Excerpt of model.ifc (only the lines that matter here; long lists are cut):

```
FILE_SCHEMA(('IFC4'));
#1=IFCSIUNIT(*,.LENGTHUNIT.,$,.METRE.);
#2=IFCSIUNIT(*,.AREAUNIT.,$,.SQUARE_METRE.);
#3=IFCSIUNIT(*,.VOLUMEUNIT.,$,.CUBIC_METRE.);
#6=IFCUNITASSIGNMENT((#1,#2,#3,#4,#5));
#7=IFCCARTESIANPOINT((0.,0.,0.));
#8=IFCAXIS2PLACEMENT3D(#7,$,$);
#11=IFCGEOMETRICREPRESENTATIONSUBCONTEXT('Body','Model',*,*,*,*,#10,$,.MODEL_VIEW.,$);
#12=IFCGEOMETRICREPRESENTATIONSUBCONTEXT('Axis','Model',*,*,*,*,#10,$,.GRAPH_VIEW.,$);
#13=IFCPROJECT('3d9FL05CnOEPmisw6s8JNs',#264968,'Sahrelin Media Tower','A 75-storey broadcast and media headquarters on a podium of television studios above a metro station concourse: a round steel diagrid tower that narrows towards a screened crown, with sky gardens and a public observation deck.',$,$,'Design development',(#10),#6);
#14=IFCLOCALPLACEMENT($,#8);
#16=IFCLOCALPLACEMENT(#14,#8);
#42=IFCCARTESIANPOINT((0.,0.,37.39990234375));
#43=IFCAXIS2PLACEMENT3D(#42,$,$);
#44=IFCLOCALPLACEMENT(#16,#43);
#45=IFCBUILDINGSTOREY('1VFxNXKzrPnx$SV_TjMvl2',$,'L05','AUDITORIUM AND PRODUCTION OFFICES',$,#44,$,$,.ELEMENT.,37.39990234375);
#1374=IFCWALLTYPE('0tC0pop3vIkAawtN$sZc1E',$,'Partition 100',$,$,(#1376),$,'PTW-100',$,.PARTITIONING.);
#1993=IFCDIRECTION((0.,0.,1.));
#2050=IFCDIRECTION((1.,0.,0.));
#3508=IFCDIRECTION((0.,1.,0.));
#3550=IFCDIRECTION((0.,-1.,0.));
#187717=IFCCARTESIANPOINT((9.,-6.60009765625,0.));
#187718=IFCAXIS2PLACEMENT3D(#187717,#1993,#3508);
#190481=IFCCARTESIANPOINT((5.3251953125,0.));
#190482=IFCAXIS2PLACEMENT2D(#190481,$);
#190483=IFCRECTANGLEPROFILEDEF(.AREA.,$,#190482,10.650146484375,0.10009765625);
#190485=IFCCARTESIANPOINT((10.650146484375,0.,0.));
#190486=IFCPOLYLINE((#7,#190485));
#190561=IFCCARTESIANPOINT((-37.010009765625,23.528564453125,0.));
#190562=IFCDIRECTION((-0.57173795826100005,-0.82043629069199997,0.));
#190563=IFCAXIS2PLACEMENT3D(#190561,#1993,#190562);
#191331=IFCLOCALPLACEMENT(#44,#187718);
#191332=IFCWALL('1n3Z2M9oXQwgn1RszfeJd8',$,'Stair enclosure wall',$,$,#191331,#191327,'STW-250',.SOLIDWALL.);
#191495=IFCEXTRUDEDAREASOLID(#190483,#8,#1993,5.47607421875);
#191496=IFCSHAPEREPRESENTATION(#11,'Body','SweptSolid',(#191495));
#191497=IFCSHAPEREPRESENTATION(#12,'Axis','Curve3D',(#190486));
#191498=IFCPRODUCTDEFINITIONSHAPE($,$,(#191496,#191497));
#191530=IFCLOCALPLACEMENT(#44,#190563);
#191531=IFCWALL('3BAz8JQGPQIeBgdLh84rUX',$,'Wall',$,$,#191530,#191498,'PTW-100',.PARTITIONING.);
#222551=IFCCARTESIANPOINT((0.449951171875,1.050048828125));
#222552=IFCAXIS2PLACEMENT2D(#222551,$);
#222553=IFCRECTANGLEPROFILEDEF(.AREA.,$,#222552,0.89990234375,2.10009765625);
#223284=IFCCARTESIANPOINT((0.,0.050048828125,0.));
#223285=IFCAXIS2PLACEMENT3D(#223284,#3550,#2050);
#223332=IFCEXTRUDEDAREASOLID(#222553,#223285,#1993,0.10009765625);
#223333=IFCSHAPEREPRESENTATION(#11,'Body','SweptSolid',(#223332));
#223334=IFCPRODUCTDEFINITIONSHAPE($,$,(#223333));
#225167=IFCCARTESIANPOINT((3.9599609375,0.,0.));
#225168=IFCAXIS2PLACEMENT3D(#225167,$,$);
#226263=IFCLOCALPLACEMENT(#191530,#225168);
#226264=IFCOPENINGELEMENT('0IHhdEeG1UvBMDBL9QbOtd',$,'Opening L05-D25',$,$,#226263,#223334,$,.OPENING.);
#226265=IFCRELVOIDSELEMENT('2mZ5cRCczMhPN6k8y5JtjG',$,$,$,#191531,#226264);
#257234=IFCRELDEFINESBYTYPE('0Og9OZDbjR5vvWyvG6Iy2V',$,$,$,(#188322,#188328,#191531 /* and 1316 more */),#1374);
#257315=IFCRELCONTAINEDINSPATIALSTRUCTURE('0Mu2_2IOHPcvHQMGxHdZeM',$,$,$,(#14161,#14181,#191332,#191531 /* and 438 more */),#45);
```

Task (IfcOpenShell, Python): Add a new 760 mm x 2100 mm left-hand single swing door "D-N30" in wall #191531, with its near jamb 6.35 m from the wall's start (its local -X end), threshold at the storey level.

```python
import numpy as np
import ifcopenshell
import ifcopenshell.api.feature
import ifcopenshell.api.geometry
import ifcopenshell.api.root
import ifcopenshell.api.spatial
import ifcopenshell.geom
import ifcopenshell.util.element
import ifcopenshell.util.placement
import ifcopenshell.util.representation
import ifcopenshell.util.shape
import ifcopenshell.util.unit

model = ifcopenshell.open("model.ifc")
unit_scale = ifcopenshell.util.unit.calculate_unit_scale(model)
settings = ifcopenshell.geom.settings()


def volume(element):
    """Net volume in cubic metres, openings subtracted."""
    shape = ifcopenshell.geom.create_shape(settings, element)
    return ifcopenshell.util.shape.get_volume(shape.geometry)


wall = model.by_guid("3BAz8JQGPQIeBgdLh84rUX")
storey = ifcopenshell.util.element.get_container(wall, ifc_class="IfcBuildingStorey")
context = ifcopenshell.util.representation.get_context(model, "Model", "Body", "MODEL_VIEW")
before = volume(wall)

width, height, from_end, sill = 0.76, 2.1, 6.35, 0.0  # metres

# The wall runs along its own X axis, and the end named is its -X end.
wall_shape = ifcopenshell.geom.create_shape(settings, wall)
x, y, z = ifcopenshell.util.shape.get_vertices(wall_shape.geometry).T
start = x.min() + from_end
face, thickness = float(y.min()), float(y.max() - y.min())
wall_matrix = ifcopenshell.util.placement.get_local_placement(wall.ObjectPlacement)
level = ifcopenshell.util.placement.get_local_placement(storey.ObjectPlacement)[2, 3]


def in_wall(x, y):
    """Placement at x, y metres in the wall's axes, at sill height."""
    matrix = wall_matrix.copy()
    matrix[:, 3] = wall_matrix @ np.array([x / unit_scale, y / unit_scale, 0.0, 1.0])
    matrix[2, 3] = level + sill / unit_scale
    return matrix


# Opening: a box that overshoots both wall faces by 50 mm.
opening = ifcopenshell.api.root.create_entity(model, ifc_class="IfcOpeningElement", predefined_type="OPENING")
box = ifcopenshell.api.geometry.add_wall_representation(
    model, context=context, length=width, height=height, thickness=thickness + 0.1
)
ifcopenshell.api.geometry.assign_representation(model, product=opening, representation=box)
ifcopenshell.api.geometry.edit_object_placement(model, product=opening, matrix=in_wall(start, face - 0.05), is_si=False)
ifcopenshell.api.feature.add_feature(model, feature=opening, element=wall)

door = ifcopenshell.api.root.create_entity(model, ifc_class="IfcDoor", name="D-N30", predefined_type="DOOR")
door.OverallWidth, door.OverallHeight = width / unit_scale, height / unit_scale
door.OperationType = "SINGLE_SWING_LEFT"
body = ifcopenshell.api.geometry.add_door_representation(
    model,
    context=context,
    overall_width=door.OverallWidth,
    overall_height=door.OverallHeight,
    operation_type="SINGLE_SWING_LEFT",
    lining_properties={"LiningDepth": thickness / unit_scale, "ThresholdDepth": thickness / unit_scale},
)
ifcopenshell.api.geometry.assign_representation(model, product=door, representation=body)
ifcopenshell.api.spatial.assign_container(model, products=[door], relating_structure=storey)
ifcopenshell.api.feature.add_filling(model, opening=opening, element=door)

# The lining spans the wall, so the door starts at the wall face.
ifcopenshell.api.geometry.edit_object_placement(model, product=door, matrix=in_wall(start, face), is_si=False)

after = volume(wall)

print(f"wall volume {before:.3f} -> {after:.3f} m3")

model.write("model-out.ifc")
```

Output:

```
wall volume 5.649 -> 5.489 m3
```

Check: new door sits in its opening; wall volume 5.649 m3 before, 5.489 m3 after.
